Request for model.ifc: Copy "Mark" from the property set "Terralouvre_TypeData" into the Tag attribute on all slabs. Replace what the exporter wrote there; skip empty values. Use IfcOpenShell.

First a look at what the model holds.

```python
import ifcopenshell
import ifcopenshell.util.element

model = ifcopenshell.open("model.ifc")
print(model.schema)
slabs = model.by_type("IfcSlab")
print(len(slabs), "slabs")
for e in slabs[:8]:
    source = ifcopenshell.util.element.get_pset(e, "Terralouvre_TypeData", "Mark")
    target = e.Tag
    print(e.id(), repr(source), repr(target), sep=" | ")
```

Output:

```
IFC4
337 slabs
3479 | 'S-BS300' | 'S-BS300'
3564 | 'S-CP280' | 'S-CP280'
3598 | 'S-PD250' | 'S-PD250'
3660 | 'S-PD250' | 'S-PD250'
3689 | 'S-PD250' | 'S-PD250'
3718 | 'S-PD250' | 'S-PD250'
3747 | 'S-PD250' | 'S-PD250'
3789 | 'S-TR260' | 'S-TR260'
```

```python
import ifcopenshell
import ifcopenshell.util.element

model = ifcopenshell.open("model.ifc")

count = 0
for e in model.by_type("IfcSlab"):
    value = ifcopenshell.util.element.get_pset(e, "Terralouvre_TypeData", "Mark")
    current = e.Tag
    if not value or not value.strip() or current == value:
        continue
    e.Tag = value
    count += 1

print(count, "slabs updated")

model.write("model_updated.ifc")
```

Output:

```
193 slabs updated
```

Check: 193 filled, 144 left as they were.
